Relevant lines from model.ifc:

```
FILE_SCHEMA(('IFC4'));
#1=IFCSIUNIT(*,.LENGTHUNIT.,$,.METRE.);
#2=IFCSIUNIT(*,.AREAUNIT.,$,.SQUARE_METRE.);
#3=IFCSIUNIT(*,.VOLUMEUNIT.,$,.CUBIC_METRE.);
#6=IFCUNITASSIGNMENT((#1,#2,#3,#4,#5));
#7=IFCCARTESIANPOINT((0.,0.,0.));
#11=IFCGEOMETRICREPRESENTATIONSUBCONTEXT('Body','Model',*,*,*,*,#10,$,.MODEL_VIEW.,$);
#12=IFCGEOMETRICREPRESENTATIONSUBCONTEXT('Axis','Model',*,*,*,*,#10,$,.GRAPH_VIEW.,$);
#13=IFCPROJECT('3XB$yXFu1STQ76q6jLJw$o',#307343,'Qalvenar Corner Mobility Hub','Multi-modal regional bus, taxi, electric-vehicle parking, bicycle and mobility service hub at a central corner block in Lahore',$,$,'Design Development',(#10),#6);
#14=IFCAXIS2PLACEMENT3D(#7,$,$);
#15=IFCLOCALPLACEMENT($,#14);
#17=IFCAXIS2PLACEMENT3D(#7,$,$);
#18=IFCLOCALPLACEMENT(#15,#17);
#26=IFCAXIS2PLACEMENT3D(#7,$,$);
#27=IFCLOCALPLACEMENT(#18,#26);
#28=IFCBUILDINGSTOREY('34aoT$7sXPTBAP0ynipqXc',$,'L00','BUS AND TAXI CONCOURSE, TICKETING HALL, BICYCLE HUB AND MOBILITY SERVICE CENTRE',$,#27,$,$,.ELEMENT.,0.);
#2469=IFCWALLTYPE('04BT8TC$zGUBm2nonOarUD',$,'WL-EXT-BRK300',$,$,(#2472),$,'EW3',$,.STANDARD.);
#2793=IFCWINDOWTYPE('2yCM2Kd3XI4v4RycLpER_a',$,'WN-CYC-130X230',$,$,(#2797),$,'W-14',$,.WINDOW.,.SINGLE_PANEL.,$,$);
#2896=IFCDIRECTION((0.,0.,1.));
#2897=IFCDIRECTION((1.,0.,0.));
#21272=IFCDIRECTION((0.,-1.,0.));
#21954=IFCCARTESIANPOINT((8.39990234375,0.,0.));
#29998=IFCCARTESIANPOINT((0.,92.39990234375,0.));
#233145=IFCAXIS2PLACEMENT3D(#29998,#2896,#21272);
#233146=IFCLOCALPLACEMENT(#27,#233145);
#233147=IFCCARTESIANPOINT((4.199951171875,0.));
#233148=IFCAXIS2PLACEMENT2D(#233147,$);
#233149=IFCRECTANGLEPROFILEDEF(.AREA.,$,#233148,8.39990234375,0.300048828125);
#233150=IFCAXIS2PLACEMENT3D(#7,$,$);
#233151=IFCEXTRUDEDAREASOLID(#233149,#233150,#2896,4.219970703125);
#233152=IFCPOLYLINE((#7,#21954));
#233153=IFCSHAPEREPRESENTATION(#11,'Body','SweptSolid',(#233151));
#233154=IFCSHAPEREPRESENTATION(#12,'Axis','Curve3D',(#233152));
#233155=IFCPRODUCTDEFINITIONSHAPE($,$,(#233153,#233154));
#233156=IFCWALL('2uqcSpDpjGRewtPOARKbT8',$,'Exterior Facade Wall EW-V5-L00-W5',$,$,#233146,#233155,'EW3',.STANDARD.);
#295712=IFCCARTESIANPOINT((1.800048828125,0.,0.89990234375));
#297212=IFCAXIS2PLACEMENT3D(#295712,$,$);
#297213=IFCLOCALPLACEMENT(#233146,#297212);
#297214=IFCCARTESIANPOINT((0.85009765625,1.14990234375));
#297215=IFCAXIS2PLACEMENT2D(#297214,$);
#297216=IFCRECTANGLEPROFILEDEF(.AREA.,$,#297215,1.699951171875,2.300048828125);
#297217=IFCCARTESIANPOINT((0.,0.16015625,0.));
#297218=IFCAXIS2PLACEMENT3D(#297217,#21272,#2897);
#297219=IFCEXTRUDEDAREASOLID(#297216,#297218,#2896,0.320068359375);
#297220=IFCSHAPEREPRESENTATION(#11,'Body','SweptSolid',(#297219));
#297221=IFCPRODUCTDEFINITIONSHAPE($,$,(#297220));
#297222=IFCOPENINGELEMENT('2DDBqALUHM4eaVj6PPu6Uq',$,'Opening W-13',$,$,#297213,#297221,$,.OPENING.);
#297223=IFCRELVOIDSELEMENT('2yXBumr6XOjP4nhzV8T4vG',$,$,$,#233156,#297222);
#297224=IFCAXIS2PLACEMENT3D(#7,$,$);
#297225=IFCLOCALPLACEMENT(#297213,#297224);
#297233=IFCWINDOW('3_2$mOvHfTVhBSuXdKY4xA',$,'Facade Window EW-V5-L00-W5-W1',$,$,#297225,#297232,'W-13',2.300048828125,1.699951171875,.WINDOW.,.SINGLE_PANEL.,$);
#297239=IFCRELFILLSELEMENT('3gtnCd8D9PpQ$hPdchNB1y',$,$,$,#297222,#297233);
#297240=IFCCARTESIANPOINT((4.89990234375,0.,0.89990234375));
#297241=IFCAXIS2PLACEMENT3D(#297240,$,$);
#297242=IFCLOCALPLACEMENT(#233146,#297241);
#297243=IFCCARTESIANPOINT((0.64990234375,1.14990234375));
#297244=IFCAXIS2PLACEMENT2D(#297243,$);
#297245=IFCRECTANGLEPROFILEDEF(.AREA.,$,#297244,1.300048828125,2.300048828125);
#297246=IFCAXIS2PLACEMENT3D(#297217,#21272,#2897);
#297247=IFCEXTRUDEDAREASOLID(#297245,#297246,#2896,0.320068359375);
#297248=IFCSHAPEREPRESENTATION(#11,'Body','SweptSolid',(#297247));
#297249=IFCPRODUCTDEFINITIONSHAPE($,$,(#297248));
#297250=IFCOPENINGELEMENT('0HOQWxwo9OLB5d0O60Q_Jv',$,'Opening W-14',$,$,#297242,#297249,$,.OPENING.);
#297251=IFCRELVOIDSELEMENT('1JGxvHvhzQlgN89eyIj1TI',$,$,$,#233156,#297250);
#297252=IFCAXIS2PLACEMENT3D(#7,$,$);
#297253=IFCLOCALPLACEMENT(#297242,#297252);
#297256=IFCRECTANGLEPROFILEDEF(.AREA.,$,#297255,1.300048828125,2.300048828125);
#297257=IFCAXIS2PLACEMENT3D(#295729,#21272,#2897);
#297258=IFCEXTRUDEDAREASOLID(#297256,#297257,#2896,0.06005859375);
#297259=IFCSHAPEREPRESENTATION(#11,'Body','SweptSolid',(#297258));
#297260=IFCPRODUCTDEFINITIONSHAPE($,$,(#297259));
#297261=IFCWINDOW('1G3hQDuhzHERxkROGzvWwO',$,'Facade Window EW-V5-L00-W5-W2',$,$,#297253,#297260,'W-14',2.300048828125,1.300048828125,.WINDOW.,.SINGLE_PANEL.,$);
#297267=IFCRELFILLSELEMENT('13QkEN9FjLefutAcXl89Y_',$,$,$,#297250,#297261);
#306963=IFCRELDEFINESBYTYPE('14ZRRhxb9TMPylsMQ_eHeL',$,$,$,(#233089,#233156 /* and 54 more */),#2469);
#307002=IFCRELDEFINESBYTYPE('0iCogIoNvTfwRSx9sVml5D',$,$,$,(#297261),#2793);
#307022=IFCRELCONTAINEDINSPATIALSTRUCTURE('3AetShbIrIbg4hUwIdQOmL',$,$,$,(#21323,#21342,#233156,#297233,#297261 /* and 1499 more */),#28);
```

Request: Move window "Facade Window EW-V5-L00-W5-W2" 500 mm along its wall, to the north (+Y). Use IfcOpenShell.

```python
import ifcopenshell
import ifcopenshell.api.geometry
import ifcopenshell.util.placement

model = ifcopenshell.open("model.ifc")

window = model.by_id(297261)
opening = window.FillsVoids[0].RelatingOpeningElement
wall = opening.VoidsElements[0].RelatingBuildingElement

wall_matrix = ifcopenshell.util.placement.get_local_placement(wall.ObjectPlacement)
shift = wall_matrix[:3, 0] * -0.5
before = ifcopenshell.util.placement.get_local_placement(window.ObjectPlacement)[:3, 3].copy()

# The window is placed relative to its opening, so it follows when the opening moves.
matrix = ifcopenshell.util.placement.get_local_placement(opening.ObjectPlacement)
matrix[:3, 3] += shift
ifcopenshell.api.geometry.edit_object_placement(
    model, product=opening, matrix=matrix, is_si=False, should_transform_children=True
)

after = ifcopenshell.util.placement.get_local_placement(window.ObjectPlacement)[:3, 3]
print("window moved by", (after - before).round(3) + 0.0)

model.write("model_edited.ifc")
```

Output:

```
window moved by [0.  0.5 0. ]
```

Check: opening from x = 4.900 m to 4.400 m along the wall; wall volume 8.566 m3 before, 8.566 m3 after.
